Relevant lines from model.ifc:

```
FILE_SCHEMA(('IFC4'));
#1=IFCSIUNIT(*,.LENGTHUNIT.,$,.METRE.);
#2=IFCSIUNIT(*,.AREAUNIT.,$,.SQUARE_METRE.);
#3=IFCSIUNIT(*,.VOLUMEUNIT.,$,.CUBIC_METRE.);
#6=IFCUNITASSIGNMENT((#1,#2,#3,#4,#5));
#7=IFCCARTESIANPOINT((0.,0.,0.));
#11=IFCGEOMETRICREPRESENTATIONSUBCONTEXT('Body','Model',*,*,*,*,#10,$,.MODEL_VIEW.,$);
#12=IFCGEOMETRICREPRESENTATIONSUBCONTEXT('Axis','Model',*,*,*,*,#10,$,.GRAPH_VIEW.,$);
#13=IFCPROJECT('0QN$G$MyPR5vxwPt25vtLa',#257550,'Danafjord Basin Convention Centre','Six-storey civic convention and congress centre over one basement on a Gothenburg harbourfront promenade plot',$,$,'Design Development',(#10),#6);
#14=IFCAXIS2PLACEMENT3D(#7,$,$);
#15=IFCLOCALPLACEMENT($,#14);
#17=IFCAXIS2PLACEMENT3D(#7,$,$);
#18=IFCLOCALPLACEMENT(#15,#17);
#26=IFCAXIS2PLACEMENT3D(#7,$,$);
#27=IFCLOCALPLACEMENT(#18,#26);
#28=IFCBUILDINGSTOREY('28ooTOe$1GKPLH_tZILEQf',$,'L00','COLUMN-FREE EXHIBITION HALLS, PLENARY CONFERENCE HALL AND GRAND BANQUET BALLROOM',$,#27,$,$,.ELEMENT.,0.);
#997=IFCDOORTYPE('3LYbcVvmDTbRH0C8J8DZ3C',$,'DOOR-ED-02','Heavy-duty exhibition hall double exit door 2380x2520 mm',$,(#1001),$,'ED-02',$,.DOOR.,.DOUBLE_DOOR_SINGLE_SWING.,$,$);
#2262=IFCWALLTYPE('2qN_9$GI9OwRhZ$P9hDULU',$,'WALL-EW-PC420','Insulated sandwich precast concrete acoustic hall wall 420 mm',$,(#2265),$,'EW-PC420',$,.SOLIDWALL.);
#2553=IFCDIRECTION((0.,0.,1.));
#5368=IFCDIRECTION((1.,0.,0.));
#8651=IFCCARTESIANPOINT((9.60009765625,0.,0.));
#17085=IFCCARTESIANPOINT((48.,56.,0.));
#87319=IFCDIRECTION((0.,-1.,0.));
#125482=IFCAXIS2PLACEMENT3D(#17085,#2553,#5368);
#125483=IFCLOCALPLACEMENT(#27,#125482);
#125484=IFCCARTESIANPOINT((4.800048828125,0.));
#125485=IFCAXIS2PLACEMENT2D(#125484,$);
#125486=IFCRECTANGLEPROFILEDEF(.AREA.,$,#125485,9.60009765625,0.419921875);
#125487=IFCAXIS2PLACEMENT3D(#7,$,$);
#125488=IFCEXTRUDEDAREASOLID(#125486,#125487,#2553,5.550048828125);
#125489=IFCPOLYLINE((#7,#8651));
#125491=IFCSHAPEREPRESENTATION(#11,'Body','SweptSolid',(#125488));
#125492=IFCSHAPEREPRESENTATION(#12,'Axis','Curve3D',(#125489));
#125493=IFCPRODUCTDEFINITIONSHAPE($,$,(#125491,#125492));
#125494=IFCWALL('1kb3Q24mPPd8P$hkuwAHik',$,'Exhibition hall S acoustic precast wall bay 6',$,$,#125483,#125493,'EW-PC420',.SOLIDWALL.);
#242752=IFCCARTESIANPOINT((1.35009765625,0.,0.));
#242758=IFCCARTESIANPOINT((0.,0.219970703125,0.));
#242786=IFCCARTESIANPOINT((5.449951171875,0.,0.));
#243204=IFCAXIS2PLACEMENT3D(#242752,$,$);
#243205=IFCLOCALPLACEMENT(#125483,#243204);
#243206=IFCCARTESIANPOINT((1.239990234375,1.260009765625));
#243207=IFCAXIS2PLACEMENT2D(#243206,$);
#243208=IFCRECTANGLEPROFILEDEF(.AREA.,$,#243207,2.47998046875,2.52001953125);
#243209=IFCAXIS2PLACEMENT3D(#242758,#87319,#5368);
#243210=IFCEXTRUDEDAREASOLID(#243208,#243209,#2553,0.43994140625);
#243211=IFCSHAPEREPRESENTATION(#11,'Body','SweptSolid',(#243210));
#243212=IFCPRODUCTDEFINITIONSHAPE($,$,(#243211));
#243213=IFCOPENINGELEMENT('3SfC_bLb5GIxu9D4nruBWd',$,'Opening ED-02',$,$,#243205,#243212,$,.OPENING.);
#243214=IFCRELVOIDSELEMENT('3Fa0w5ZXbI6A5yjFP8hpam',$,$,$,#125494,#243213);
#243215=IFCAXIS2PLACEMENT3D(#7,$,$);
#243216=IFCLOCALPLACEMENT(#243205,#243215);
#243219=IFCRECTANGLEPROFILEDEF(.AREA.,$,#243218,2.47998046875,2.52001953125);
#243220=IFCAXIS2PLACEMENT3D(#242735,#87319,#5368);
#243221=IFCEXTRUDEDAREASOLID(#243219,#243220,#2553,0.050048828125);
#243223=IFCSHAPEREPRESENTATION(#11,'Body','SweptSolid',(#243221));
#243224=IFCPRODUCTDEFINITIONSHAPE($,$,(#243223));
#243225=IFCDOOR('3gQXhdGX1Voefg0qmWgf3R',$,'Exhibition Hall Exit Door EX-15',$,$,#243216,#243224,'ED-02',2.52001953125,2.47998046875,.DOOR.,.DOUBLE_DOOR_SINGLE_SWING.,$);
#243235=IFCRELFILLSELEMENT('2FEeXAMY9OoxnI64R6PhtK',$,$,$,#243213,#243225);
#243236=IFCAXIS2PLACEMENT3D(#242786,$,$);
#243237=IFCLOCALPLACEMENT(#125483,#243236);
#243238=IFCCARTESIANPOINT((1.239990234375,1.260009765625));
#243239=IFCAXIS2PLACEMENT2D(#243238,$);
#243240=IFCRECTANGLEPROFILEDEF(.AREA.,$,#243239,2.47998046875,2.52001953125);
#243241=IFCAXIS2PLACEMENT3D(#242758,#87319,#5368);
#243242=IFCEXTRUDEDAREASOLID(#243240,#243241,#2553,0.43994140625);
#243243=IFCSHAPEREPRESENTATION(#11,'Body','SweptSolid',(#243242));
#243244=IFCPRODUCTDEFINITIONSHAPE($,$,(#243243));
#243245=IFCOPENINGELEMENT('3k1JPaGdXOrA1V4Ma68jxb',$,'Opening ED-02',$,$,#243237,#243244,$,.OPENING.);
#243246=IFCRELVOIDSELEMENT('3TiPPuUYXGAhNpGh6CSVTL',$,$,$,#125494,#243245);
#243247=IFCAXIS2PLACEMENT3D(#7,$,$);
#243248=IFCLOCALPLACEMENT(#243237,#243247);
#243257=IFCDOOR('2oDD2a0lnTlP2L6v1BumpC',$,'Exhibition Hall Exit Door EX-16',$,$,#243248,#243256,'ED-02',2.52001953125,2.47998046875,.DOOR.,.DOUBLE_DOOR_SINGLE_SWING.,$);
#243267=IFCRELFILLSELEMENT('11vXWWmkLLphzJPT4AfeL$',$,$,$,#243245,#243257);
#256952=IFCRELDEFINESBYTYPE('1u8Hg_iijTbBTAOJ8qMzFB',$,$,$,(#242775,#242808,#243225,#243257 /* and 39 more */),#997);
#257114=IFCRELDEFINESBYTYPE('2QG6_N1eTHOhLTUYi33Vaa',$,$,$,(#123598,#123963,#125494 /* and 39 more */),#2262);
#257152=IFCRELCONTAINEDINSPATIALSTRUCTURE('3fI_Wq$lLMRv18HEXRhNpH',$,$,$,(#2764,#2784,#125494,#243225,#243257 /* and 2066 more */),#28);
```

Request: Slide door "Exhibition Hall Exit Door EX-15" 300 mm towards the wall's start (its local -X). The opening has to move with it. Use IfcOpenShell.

```python
import ifcopenshell
import ifcopenshell.api.geometry
import ifcopenshell.util.placement
import ifcopenshell.util.unit

model = ifcopenshell.open("model.ifc")
unit_scale = ifcopenshell.util.unit.calculate_unit_scale(model)

door = model.by_id(243225)
opening = door.FillsVoids[0].RelatingOpeningElement
wall = opening.VoidsElements[0].RelatingBuildingElement

wall_matrix = ifcopenshell.util.placement.get_local_placement(wall.ObjectPlacement)
shift = wall_matrix[:3, 0] * -0.3 / unit_scale
before = ifcopenshell.util.placement.get_local_placement(door.ObjectPlacement)[:3, 3].copy()

# The door is placed relative to its opening, so it follows when the opening moves.
matrix = ifcopenshell.util.placement.get_local_placement(opening.ObjectPlacement)
matrix[:3, 3] += shift
ifcopenshell.api.geometry.edit_object_placement(
    model, product=opening, matrix=matrix, is_si=False, should_transform_children=True
)

after = ifcopenshell.util.placement.get_local_placement(door.ObjectPlacement)[:3, 3]
print("door moved by", (after - before).round(3) + 0.0)

model.write("model-out.ifc")
```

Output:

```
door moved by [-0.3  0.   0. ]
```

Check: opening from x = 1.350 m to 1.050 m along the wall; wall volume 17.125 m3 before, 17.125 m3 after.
